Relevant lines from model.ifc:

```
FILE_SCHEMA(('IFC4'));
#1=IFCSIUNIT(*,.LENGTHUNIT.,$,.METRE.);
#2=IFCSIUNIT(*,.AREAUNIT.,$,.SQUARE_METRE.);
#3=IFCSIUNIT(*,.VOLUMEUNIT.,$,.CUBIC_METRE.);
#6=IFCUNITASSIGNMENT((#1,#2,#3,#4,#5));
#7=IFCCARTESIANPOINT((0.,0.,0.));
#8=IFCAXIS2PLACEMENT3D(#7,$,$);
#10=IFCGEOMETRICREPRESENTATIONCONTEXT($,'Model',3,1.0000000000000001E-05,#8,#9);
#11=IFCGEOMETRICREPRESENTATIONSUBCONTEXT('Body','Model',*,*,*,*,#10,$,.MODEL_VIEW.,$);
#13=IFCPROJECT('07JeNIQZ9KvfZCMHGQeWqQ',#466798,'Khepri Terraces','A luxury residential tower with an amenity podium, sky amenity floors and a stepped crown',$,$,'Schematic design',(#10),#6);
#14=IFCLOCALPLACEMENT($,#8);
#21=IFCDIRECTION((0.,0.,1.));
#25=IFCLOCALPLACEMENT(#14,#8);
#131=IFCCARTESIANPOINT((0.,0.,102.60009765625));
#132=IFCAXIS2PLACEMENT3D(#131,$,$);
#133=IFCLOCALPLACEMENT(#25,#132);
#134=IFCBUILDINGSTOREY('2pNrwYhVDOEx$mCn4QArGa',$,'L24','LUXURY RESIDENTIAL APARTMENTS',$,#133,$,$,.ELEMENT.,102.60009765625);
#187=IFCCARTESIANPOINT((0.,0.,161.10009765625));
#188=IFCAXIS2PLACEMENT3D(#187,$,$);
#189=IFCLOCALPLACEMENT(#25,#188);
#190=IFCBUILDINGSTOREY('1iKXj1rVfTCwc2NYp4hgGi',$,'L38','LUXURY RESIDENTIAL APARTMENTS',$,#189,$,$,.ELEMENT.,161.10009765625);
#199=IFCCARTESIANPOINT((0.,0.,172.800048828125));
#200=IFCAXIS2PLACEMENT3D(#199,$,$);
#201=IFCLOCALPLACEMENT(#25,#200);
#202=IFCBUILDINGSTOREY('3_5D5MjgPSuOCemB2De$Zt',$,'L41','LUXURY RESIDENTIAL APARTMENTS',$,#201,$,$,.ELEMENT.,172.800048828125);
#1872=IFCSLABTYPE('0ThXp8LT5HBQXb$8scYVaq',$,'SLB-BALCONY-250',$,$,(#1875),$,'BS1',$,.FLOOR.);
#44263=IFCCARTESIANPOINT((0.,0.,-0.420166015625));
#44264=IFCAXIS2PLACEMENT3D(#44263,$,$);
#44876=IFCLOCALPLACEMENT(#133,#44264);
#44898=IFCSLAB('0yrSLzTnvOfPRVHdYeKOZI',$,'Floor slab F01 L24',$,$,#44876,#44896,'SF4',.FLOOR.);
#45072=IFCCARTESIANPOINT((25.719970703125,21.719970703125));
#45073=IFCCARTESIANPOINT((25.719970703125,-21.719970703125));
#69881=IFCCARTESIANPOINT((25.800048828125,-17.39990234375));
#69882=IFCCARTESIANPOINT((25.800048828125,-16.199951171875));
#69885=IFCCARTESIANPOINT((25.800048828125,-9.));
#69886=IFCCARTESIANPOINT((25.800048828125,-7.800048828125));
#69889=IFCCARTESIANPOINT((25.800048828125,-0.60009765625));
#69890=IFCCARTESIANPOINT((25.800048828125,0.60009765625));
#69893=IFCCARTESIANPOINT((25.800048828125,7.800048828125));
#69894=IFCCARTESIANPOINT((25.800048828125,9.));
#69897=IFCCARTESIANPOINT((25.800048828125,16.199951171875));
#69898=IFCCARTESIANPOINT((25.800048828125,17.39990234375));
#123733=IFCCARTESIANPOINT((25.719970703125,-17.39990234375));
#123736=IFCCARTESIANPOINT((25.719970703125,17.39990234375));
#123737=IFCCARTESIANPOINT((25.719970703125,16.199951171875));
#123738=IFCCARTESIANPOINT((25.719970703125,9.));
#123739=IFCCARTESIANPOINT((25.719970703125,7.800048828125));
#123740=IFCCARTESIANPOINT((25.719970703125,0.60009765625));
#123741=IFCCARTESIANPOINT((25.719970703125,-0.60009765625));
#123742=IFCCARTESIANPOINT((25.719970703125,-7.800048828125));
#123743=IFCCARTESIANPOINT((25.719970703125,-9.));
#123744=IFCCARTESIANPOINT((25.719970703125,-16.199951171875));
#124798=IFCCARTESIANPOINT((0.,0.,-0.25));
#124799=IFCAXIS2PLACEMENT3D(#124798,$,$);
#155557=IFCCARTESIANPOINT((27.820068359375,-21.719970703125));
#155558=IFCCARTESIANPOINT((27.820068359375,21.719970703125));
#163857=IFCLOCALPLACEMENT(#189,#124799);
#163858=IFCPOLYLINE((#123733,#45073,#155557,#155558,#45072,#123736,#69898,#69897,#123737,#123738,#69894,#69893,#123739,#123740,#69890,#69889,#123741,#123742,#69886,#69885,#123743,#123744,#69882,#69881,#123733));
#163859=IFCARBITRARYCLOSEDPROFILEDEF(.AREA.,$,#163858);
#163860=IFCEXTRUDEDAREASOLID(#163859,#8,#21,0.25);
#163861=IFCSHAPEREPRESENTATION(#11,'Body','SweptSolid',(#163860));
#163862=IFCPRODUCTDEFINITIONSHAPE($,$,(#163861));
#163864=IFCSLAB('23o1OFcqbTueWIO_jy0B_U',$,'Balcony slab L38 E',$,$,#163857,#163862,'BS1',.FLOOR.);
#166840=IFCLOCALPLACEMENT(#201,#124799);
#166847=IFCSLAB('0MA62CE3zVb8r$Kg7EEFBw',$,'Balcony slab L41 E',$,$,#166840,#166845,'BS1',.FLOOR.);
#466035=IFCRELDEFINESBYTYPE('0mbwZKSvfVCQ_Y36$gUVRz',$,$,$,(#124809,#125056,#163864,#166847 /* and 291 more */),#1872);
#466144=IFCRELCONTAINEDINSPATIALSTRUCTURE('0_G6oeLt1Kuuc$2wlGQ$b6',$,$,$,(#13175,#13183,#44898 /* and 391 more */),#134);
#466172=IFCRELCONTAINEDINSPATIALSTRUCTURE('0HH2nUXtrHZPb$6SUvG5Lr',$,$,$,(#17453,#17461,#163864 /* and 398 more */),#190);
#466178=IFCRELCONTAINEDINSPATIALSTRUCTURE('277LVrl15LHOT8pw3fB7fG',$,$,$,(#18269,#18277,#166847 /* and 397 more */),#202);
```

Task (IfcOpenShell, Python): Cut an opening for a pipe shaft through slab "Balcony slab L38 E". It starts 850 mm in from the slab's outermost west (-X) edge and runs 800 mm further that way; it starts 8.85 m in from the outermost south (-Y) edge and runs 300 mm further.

```python
import numpy as np
import ifcopenshell
import ifcopenshell.api.feature
import ifcopenshell.api.geometry
import ifcopenshell.api.root
import ifcopenshell.geom
import ifcopenshell.util.placement
import ifcopenshell.util.representation
import ifcopenshell.util.shape
import ifcopenshell.util.unit

model = ifcopenshell.open("model.ifc")
unit_scale = ifcopenshell.util.unit.calculate_unit_scale(model)
settings = ifcopenshell.geom.settings()


def volume(element):
    """Net volume in cubic metres, openings subtracted."""
    shape = ifcopenshell.geom.create_shape(settings, element)
    return ifcopenshell.util.shape.get_volume(shape.geometry)


slab = model.by_guid("23o1OFcqbTueWIO_jy0B_U")
before = volume(slab)

# Extent in the slab's own axes, in metres. The edges named are its -X and -Y sides.
slab_shape = ifcopenshell.geom.create_shape(settings, slab)
vertices = ifcopenshell.util.shape.get_vertices(slab_shape.geometry)
x_min, y_min, bottom = vertices.min(axis=0)
top = vertices[:, 2].max()

opening = ifcopenshell.api.root.create_entity(model, ifc_class="IfcOpeningElement", name="Pipe shaft opening", predefined_type="OPENING")
context = ifcopenshell.util.representation.get_context(model, "Model", "Body", "MODEL_VIEW")
width, depth = 0.8, 0.3
outline = [(0.0, 0.0), (width, 0.0), (width, depth), (0.0, depth), (0.0, 0.0)]
# Overshoot both faces by 50 mm so the cut is clean.
shape = ifcopenshell.api.geometry.add_slab_representation(
    model, context=context, depth=top - bottom + 0.1, polyline=outline
)
ifcopenshell.api.geometry.assign_representation(model, product=opening, representation=shape)

matrix = ifcopenshell.util.placement.get_local_placement(slab.ObjectPlacement)
matrix[:, 3] = matrix @ np.append(np.array([x_min + 0.85, y_min + 8.85, bottom - 0.05]) / unit_scale, 1.0)
ifcopenshell.api.geometry.edit_object_placement(model, product=opening, matrix=matrix, is_si=False)
ifcopenshell.api.feature.add_feature(model, feature=opening, element=slab)

after = volume(slab)

print(f"slab volume {before:.3f} -> {after:.3f} m3")

model.write("model_rev.ifc")
```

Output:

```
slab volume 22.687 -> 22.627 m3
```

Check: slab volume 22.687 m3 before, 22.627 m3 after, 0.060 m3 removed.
